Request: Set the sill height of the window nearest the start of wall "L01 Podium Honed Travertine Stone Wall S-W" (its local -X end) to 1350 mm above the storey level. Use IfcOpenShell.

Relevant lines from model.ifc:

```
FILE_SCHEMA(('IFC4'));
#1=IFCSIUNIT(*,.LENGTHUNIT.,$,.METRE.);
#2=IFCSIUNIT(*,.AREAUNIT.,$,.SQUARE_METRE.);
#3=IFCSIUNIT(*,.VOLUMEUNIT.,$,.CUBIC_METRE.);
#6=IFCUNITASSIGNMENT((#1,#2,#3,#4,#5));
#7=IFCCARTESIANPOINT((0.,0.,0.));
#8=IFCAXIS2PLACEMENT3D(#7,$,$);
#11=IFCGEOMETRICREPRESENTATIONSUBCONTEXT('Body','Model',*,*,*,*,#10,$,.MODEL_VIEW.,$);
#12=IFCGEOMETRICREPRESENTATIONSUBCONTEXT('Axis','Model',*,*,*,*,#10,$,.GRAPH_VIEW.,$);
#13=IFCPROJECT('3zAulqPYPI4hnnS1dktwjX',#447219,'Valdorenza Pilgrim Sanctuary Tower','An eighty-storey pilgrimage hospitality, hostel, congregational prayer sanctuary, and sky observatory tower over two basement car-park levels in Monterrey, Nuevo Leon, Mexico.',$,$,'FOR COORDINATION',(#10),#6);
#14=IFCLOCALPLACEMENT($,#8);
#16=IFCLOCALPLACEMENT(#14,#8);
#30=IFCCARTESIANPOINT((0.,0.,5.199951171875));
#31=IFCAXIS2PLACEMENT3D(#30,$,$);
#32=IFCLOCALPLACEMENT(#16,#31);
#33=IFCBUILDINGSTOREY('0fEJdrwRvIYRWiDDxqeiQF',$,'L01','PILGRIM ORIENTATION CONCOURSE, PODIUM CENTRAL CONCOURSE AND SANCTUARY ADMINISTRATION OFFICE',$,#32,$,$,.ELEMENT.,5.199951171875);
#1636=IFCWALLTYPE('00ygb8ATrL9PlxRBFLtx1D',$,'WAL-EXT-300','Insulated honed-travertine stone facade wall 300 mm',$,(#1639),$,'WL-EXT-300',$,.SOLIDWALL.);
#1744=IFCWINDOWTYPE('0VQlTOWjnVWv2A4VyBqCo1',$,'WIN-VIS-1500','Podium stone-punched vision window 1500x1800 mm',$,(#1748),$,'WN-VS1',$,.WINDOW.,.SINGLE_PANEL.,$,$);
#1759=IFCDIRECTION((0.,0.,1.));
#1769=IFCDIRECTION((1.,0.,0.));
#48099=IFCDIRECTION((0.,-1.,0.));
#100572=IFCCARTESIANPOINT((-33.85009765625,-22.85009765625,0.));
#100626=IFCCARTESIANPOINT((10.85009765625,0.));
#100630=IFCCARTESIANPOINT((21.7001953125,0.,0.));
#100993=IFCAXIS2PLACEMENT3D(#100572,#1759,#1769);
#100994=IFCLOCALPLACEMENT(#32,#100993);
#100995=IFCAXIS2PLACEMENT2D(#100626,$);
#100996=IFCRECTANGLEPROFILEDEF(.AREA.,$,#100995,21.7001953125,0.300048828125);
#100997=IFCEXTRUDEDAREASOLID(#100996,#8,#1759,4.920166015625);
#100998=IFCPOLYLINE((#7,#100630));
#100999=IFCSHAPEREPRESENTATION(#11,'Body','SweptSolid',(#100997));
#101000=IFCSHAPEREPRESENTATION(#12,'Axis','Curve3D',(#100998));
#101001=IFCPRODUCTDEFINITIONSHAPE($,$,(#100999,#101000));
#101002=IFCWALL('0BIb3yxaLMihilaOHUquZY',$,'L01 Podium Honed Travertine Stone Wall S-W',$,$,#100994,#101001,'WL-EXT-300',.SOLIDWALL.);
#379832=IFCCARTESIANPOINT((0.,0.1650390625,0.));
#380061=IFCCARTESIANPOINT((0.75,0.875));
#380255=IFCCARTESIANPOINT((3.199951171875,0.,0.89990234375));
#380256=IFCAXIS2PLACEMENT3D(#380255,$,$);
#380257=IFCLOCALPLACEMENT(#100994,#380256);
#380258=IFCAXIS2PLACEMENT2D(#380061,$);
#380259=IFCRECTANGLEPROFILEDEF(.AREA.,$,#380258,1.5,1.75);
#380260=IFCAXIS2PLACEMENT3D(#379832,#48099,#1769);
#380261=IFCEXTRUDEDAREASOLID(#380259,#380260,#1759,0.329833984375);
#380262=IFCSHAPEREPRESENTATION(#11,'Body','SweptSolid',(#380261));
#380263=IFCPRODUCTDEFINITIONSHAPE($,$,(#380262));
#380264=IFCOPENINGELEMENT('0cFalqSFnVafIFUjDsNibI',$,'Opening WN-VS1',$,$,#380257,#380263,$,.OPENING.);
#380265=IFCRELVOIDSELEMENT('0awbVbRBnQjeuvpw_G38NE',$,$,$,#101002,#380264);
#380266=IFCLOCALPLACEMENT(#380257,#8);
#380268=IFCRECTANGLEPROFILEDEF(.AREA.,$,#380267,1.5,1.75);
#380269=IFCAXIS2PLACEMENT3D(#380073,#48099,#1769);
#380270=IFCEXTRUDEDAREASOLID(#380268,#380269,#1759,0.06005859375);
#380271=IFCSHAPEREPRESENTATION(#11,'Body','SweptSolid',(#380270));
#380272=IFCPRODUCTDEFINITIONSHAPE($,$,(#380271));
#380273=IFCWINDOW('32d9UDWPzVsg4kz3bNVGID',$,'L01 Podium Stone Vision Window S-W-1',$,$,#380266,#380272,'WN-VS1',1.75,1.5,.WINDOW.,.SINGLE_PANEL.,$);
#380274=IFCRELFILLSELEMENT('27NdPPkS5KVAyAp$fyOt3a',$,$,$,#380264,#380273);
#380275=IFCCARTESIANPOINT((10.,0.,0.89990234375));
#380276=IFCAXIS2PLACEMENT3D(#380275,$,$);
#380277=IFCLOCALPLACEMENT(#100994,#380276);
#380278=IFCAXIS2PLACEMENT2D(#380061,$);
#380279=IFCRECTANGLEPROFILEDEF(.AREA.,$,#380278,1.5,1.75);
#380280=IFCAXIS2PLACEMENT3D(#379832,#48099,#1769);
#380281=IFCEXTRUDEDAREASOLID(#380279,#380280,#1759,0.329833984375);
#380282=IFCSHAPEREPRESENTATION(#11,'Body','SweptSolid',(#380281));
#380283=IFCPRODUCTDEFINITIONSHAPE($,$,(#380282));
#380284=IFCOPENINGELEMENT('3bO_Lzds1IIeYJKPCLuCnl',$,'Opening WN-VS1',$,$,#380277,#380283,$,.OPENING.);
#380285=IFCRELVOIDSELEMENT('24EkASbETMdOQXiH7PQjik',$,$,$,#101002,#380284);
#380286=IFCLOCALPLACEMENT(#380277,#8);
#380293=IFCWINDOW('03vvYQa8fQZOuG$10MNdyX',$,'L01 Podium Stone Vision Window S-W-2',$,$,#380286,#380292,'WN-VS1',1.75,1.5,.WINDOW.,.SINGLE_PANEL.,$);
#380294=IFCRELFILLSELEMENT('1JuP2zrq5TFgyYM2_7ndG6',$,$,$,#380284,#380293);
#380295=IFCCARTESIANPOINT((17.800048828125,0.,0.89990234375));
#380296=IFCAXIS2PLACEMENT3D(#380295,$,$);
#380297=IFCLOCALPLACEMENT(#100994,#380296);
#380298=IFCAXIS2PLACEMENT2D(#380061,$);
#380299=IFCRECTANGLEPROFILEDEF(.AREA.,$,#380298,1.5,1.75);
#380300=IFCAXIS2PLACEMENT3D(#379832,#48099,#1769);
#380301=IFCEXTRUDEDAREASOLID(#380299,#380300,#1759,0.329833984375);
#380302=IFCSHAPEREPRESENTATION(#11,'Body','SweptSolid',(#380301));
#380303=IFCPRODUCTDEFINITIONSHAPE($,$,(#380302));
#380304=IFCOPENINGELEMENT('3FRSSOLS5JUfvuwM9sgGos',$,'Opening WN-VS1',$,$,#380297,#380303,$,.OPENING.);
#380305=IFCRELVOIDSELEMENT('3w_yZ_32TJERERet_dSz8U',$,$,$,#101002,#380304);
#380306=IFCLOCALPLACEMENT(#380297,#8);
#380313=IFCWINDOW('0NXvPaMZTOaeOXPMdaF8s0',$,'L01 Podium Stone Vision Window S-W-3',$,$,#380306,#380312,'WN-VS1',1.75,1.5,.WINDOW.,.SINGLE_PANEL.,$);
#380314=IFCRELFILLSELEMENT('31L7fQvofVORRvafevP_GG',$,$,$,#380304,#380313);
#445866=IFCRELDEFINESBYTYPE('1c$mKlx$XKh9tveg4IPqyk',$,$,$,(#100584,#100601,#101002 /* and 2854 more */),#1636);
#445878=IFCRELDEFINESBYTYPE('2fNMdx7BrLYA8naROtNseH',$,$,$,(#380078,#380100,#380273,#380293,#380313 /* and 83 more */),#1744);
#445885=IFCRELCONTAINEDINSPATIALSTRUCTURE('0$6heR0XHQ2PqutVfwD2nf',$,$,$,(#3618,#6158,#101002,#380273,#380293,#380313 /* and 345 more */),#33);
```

```python
import numpy as np
import ifcopenshell
import ifcopenshell.api.geometry
import ifcopenshell.geom
import ifcopenshell.util.element
import ifcopenshell.util.placement
import ifcopenshell.util.shape
import ifcopenshell.util.unit

model = ifcopenshell.open("model.ifc")
unit_scale = ifcopenshell.util.unit.calculate_unit_scale(model)

window = model.by_guid("32d9UDWPzVsg4kz3bNVGID")
opening = window.FillsVoids[0].RelatingOpeningElement
storey = ifcopenshell.util.element.get_container(window, ifc_class="IfcBuildingStorey")
level = ifcopenshell.util.placement.get_local_placement(storey.ObjectPlacement)[2, 3]

# The opening's origin need not be at the sill, so measure its lowest point.
shape = ifcopenshell.geom.create_shape(ifcopenshell.geom.settings(), opening)
bottom = ifcopenshell.util.shape.get_shape_bottom_elevation(shape, shape.geometry) / unit_scale
dz = level + 1.35 - bottom

shift = np.array([0.0, 0.0, dz])
# The window is placed relative to its opening, so it follows when the opening moves.
matrix = ifcopenshell.util.placement.get_local_placement(opening.ObjectPlacement)
matrix[:3, 3] += shift
ifcopenshell.api.geometry.edit_object_placement(
    model, product=opening, matrix=matrix, is_si=False, should_transform_children=True
)

print(f"moved by {dz * unit_scale:+.3f} m")

model.write("model_v2.ifc")
```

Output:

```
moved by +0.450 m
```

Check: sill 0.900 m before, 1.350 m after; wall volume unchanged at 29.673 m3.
